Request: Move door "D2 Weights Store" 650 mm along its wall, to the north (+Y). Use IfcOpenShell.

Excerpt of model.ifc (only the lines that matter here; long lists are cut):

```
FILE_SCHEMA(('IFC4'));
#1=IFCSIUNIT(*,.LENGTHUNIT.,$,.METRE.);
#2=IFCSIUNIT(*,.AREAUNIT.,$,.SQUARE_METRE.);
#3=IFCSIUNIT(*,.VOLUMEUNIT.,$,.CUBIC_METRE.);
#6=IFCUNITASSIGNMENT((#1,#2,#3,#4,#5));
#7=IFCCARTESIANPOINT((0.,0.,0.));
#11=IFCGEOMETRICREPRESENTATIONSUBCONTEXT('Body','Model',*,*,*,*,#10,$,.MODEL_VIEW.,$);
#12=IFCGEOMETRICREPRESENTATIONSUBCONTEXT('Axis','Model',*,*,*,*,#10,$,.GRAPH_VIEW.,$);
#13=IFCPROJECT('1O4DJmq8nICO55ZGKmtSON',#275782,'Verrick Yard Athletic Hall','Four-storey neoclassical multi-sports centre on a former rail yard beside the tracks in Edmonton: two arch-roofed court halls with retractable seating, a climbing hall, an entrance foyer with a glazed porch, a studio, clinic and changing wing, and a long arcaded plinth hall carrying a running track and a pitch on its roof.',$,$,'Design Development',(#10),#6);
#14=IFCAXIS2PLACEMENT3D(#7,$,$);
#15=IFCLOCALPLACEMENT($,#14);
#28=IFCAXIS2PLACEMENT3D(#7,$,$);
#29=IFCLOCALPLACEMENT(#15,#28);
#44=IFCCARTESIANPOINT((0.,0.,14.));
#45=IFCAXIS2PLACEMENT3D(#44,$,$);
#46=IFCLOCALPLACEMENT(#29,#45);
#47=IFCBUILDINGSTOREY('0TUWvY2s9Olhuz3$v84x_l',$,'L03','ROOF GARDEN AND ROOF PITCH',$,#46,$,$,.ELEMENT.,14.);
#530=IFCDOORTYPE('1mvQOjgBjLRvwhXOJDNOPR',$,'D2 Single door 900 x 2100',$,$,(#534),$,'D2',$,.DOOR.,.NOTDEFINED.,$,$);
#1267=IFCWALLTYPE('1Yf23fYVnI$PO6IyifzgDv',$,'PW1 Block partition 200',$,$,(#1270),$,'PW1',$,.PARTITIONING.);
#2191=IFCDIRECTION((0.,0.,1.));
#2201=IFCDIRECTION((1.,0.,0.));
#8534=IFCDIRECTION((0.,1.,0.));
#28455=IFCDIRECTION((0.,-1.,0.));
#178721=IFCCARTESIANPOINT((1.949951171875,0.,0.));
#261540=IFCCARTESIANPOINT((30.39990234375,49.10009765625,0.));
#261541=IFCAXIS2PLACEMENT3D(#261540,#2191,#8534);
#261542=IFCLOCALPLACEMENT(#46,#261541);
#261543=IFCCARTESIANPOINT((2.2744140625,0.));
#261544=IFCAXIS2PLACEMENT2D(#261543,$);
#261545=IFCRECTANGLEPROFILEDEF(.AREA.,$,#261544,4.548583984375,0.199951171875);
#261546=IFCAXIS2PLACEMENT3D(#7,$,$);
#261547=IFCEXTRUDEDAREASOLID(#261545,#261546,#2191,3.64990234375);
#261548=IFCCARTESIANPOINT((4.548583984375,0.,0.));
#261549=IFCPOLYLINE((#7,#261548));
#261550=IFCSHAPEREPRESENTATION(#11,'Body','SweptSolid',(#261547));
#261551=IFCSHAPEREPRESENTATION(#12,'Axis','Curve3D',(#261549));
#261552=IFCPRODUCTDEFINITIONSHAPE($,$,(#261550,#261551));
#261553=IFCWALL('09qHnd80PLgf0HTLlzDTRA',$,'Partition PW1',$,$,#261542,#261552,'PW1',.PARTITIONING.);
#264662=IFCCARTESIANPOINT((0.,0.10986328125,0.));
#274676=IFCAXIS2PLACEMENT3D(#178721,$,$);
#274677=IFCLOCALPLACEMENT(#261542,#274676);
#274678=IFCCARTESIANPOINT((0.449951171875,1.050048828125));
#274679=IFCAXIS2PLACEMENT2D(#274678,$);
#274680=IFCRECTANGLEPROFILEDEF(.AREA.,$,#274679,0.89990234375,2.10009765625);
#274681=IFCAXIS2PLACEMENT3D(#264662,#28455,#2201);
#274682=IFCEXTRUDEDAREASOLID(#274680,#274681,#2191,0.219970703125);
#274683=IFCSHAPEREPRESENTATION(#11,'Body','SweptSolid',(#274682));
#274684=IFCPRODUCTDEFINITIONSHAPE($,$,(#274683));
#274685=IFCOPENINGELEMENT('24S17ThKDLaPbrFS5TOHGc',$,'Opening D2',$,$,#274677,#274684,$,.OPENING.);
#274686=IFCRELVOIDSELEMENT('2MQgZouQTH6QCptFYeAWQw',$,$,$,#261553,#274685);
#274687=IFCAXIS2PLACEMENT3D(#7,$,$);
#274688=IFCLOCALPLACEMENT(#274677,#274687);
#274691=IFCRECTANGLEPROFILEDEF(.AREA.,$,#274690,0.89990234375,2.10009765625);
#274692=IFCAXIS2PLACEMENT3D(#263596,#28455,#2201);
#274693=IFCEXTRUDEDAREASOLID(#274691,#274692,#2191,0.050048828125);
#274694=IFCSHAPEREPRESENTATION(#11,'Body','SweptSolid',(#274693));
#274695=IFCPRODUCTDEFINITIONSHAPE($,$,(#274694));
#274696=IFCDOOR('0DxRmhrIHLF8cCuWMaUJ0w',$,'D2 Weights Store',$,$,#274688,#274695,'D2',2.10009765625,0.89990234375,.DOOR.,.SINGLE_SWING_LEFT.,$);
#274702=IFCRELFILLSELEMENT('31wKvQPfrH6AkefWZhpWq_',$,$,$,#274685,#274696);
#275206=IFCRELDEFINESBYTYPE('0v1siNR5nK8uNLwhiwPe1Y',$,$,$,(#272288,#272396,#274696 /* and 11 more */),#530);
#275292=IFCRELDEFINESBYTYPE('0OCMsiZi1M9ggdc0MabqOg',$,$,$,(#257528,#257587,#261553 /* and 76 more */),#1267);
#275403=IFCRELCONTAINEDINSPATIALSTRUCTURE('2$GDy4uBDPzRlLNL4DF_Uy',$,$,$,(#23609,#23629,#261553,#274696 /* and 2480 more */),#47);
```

```python
import ifcopenshell
import ifcopenshell.api.geometry
import ifcopenshell.util.placement

model = ifcopenshell.open("model.ifc")

door = model.by_guid("0DxRmhrIHLF8cCuWMaUJ0w")
opening = door.FillsVoids[0].RelatingOpeningElement
wall = opening.VoidsElements[0].RelatingBuildingElement

wall_matrix = ifcopenshell.util.placement.get_local_placement(wall.ObjectPlacement)
shift = wall_matrix[:3, 0] * 0.65
before = ifcopenshell.util.placement.get_local_placement(door.ObjectPlacement)[:3, 3].copy()

# The door is placed relative to its opening, so it follows when the opening moves.
matrix = ifcopenshell.util.placement.get_local_placement(opening.ObjectPlacement)
matrix[:3, 3] += shift
ifcopenshell.api.geometry.edit_object_placement(
    model, product=opening, matrix=matrix, is_si=False, should_transform_children=True
)

after = ifcopenshell.util.placement.get_local_placement(door.ObjectPlacement)[:3, 3]
print("door moved by", (after - before).round(3) + 0.0)

model.write("model-out.ifc")
```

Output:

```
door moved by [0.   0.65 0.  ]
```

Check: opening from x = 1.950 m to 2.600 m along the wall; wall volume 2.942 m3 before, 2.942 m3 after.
